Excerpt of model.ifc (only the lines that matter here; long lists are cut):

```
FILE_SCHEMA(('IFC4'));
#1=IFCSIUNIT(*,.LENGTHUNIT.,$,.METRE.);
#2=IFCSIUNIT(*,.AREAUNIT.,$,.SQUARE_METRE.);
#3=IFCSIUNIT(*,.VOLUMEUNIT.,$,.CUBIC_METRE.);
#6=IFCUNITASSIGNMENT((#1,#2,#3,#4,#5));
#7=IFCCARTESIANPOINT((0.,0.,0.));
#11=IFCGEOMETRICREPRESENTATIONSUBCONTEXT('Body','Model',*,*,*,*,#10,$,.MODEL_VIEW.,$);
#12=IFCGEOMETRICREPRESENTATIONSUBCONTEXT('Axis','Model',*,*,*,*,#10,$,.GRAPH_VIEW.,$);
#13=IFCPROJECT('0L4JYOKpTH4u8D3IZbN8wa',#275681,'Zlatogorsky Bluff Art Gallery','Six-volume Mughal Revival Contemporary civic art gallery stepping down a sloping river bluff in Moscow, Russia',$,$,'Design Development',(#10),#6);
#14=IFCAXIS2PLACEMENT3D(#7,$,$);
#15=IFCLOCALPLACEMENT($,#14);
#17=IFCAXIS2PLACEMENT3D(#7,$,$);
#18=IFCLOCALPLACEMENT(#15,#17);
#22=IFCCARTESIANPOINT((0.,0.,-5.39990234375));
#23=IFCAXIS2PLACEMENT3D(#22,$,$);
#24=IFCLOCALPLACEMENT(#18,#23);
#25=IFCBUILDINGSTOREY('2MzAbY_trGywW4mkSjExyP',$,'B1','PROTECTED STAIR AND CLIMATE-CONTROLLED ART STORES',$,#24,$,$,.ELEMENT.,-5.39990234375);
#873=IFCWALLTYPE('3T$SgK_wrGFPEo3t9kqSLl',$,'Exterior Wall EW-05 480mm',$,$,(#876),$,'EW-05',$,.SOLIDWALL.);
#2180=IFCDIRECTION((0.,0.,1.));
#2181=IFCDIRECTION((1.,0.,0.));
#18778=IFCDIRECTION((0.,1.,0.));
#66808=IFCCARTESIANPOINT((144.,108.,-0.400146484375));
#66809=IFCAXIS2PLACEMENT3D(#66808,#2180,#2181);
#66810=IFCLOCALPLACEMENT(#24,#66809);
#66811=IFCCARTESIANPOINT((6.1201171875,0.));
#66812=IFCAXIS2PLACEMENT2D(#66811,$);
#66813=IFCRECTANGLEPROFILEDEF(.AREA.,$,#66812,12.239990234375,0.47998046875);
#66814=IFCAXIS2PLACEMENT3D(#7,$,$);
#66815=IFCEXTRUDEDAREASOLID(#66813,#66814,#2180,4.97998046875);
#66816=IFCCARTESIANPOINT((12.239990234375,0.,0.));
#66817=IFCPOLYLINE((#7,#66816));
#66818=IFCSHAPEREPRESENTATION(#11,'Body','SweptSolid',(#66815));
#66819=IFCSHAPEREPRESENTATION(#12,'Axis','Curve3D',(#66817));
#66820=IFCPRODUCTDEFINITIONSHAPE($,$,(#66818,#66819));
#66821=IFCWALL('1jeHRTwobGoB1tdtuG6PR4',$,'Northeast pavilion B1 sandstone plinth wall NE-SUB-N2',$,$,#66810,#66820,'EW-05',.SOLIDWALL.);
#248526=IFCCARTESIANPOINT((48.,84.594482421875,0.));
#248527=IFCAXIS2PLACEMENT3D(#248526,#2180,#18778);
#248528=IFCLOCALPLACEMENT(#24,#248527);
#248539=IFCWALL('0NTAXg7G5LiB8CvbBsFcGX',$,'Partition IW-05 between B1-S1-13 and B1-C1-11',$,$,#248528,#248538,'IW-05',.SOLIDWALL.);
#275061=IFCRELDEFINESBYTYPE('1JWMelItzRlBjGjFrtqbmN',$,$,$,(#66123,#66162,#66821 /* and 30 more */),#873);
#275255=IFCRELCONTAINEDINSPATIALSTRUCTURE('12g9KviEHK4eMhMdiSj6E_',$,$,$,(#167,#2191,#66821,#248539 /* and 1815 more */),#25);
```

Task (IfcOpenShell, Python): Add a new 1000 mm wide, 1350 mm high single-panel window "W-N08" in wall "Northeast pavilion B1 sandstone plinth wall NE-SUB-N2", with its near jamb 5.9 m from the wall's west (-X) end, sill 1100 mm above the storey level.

```python
import numpy as np
import ifcopenshell
import ifcopenshell.api.feature
import ifcopenshell.api.geometry
import ifcopenshell.api.root
import ifcopenshell.api.spatial
import ifcopenshell.geom
import ifcopenshell.util.element
import ifcopenshell.util.placement
import ifcopenshell.util.representation
import ifcopenshell.util.shape
import ifcopenshell.util.unit

model = ifcopenshell.open("model.ifc")
unit_scale = ifcopenshell.util.unit.calculate_unit_scale(model)
settings = ifcopenshell.geom.settings()


def volume(element):
    """Net volume in cubic metres, openings subtracted."""
    shape = ifcopenshell.geom.create_shape(settings, element)
    return ifcopenshell.util.shape.get_volume(shape.geometry)


wall = model.by_guid("1jeHRTwobGoB1tdtuG6PR4")
storey = ifcopenshell.util.element.get_container(wall, ifc_class="IfcBuildingStorey")
context = ifcopenshell.util.representation.get_context(model, "Model", "Body", "MODEL_VIEW")
before = volume(wall)

width, height, from_end, sill = 1, 1.35, 5.9, 1.1  # metres

# The wall runs along its own X axis, and the end named is its -X end.
wall_shape = ifcopenshell.geom.create_shape(settings, wall)
x, y, z = ifcopenshell.util.shape.get_vertices(wall_shape.geometry).T
start = x.min() + from_end
face, thickness = float(y.min()), float(y.max() - y.min())
wall_matrix = ifcopenshell.util.placement.get_local_placement(wall.ObjectPlacement)
level = ifcopenshell.util.placement.get_local_placement(storey.ObjectPlacement)[2, 3]


def in_wall(x, y):
    """Placement at x, y metres in the wall's axes, at sill height."""
    matrix = wall_matrix.copy()
    matrix[:, 3] = wall_matrix @ np.array([x / unit_scale, y / unit_scale, 0.0, 1.0])
    matrix[2, 3] = level + sill / unit_scale
    return matrix


# Opening: a box that overshoots both wall faces by 50 mm.
opening = ifcopenshell.api.root.create_entity(model, ifc_class="IfcOpeningElement", predefined_type="OPENING")
box = ifcopenshell.api.geometry.add_wall_representation(
    model, context=context, length=width, height=height, thickness=thickness + 0.1
)
ifcopenshell.api.geometry.assign_representation(model, product=opening, representation=box)
ifcopenshell.api.geometry.edit_object_placement(model, product=opening, matrix=in_wall(start, face - 0.05), is_si=False)
ifcopenshell.api.feature.add_feature(model, feature=opening, element=wall)

window = ifcopenshell.api.root.create_entity(model, ifc_class="IfcWindow", name="W-N08", predefined_type="WINDOW")
window.OverallWidth, window.OverallHeight = width / unit_scale, height / unit_scale
window.PartitioningType = "SINGLE_PANEL"
body = ifcopenshell.api.geometry.add_window_representation(
    model,
    context=context,
    overall_width=window.OverallWidth,
    overall_height=window.OverallHeight,
    partition_type="SINGLE_PANEL",
)
ifcopenshell.api.geometry.assign_representation(model, product=window, representation=body)
ifcopenshell.api.spatial.assign_container(model, products=[window], relating_structure=storey)
ifcopenshell.api.feature.add_filling(model, opening=opening, element=window)

# Centre the window in the wall's thickness.
ifcopenshell.api.geometry.edit_object_placement(model, product=window, matrix=in_wall(start, face), is_si=False)
window_shape = ifcopenshell.geom.create_shape(settings, window)
depth = ifcopenshell.util.shape.get_vertices(window_shape.geometry)[:, 1]
offset = face + thickness / 2 - (depth.min() + depth.max()) / 2
ifcopenshell.api.geometry.edit_object_placement(model, product=window, matrix=in_wall(start, offset), is_si=False)

after = volume(wall)

print(f"wall volume {before:.3f} -> {after:.3f} m3")

model.write("model-out.ifc")
```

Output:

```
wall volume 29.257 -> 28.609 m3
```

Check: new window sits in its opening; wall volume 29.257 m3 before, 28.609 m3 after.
